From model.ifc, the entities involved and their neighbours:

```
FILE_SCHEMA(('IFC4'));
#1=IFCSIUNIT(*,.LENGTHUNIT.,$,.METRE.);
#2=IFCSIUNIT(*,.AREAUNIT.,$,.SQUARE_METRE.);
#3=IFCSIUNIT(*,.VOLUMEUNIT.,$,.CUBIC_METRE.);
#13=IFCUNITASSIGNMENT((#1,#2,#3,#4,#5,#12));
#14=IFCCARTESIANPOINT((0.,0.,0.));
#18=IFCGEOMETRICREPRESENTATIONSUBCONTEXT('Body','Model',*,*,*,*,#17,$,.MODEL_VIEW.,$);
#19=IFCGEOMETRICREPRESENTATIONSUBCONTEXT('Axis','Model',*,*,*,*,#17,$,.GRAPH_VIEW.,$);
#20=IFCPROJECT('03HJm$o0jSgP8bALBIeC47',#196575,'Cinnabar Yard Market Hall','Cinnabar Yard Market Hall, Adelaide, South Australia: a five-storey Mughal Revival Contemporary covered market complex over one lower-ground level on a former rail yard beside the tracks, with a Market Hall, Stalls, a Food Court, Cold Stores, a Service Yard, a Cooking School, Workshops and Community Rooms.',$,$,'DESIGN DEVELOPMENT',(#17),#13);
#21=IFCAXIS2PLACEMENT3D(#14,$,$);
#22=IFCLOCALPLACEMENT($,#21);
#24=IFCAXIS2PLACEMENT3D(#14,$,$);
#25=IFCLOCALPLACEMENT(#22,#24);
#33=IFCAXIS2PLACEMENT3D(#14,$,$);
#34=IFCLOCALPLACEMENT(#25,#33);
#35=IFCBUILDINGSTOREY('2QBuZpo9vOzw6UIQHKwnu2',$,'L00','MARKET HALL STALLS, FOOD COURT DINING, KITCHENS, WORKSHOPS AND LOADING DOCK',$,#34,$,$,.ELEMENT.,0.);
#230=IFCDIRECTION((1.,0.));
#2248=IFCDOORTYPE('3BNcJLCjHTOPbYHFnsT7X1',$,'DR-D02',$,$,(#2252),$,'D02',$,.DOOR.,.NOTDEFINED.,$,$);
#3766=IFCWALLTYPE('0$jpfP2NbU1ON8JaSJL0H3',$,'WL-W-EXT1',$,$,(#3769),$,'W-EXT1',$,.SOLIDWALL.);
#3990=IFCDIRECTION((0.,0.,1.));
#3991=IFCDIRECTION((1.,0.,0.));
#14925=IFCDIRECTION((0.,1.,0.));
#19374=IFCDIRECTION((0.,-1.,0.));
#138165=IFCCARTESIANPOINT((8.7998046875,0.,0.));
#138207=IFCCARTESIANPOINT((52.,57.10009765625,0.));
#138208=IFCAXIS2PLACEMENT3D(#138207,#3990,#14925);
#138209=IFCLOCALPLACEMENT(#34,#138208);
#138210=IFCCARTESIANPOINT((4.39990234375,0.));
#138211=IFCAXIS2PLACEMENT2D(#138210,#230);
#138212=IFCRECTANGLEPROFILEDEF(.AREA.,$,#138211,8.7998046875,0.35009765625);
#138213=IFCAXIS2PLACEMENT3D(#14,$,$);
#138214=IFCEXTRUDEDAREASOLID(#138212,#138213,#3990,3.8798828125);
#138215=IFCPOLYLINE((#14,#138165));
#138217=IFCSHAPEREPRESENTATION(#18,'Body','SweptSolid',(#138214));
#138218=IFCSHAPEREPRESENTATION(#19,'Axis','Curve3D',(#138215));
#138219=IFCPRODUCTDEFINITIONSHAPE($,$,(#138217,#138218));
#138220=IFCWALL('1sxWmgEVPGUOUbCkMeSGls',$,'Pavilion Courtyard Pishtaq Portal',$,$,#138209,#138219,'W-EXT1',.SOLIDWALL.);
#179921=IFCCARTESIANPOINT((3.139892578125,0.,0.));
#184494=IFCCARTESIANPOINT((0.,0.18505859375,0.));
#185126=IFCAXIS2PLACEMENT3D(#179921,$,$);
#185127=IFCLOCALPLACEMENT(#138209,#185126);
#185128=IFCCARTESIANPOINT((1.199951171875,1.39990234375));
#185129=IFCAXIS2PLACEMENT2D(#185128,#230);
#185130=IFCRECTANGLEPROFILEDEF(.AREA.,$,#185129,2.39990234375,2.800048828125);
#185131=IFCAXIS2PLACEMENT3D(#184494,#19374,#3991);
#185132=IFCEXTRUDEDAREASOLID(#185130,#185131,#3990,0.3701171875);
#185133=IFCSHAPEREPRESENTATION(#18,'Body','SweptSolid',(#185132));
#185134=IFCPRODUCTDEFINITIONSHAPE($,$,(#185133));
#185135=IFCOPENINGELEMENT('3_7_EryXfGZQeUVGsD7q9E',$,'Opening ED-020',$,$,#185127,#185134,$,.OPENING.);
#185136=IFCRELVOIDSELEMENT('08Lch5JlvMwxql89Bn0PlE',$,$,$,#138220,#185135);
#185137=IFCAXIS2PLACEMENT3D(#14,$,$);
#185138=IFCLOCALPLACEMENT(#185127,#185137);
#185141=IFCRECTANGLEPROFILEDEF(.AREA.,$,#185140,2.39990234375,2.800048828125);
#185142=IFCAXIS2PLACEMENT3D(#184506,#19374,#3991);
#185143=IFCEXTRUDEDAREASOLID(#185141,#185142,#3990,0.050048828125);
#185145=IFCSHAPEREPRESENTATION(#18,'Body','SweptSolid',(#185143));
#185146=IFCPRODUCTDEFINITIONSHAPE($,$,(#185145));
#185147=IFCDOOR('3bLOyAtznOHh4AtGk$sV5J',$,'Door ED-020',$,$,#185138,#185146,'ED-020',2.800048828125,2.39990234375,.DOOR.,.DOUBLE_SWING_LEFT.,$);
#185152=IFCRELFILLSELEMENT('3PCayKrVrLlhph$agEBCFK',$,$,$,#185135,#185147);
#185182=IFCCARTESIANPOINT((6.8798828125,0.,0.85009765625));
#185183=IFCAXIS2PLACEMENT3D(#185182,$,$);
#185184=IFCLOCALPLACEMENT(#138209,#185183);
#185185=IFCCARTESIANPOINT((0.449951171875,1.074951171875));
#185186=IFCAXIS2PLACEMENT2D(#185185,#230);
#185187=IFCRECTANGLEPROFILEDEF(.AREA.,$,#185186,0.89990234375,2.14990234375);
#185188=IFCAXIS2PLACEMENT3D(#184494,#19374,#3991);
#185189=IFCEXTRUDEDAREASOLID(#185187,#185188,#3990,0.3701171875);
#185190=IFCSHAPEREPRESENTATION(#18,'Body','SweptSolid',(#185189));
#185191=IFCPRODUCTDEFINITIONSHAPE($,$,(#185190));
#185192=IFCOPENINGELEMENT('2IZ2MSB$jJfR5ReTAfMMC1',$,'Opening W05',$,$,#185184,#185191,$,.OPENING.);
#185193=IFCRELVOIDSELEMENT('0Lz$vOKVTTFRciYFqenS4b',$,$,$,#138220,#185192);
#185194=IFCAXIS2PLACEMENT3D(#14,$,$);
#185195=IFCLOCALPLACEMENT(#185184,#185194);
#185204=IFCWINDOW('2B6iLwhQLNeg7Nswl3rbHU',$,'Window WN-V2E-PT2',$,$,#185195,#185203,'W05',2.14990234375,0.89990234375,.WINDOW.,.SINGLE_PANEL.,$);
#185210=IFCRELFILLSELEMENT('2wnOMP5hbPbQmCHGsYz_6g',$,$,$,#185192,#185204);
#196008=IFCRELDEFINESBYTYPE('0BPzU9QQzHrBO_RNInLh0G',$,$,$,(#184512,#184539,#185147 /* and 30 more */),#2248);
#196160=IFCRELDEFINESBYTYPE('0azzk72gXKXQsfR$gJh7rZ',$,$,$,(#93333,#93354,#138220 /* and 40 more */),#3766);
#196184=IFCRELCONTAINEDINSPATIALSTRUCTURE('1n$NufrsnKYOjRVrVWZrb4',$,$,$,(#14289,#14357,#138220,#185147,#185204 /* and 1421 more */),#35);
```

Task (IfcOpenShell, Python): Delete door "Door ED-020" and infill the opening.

```python
import ifcopenshell
import ifcopenshell.api.feature
import ifcopenshell.api.root
import ifcopenshell.geom
import ifcopenshell.util.shape

model = ifcopenshell.open("model.ifc")
settings = ifcopenshell.geom.settings()


def volume(element):
    """Net volume in cubic metres, openings subtracted."""
    shape = ifcopenshell.geom.create_shape(settings, element)
    return ifcopenshell.util.shape.get_volume(shape.geometry)


door = model.by_guid("3bLOyAtznOHh4AtGk$sV5J")
opening = door.FillsVoids[0].RelatingOpeningElement
wall = opening.VoidsElements[0].RelatingBuildingElement
before = volume(wall)

ifcopenshell.api.root.remove_product(model, product=door)
ifcopenshell.api.feature.remove_feature(model, feature=opening)

after = volume(wall)

print(f"wall volume {before:.3f} -> {after:.3f} m3")

model.write("model_v2.ifc")
```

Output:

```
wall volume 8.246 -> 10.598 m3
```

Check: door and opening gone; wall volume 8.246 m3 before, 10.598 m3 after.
